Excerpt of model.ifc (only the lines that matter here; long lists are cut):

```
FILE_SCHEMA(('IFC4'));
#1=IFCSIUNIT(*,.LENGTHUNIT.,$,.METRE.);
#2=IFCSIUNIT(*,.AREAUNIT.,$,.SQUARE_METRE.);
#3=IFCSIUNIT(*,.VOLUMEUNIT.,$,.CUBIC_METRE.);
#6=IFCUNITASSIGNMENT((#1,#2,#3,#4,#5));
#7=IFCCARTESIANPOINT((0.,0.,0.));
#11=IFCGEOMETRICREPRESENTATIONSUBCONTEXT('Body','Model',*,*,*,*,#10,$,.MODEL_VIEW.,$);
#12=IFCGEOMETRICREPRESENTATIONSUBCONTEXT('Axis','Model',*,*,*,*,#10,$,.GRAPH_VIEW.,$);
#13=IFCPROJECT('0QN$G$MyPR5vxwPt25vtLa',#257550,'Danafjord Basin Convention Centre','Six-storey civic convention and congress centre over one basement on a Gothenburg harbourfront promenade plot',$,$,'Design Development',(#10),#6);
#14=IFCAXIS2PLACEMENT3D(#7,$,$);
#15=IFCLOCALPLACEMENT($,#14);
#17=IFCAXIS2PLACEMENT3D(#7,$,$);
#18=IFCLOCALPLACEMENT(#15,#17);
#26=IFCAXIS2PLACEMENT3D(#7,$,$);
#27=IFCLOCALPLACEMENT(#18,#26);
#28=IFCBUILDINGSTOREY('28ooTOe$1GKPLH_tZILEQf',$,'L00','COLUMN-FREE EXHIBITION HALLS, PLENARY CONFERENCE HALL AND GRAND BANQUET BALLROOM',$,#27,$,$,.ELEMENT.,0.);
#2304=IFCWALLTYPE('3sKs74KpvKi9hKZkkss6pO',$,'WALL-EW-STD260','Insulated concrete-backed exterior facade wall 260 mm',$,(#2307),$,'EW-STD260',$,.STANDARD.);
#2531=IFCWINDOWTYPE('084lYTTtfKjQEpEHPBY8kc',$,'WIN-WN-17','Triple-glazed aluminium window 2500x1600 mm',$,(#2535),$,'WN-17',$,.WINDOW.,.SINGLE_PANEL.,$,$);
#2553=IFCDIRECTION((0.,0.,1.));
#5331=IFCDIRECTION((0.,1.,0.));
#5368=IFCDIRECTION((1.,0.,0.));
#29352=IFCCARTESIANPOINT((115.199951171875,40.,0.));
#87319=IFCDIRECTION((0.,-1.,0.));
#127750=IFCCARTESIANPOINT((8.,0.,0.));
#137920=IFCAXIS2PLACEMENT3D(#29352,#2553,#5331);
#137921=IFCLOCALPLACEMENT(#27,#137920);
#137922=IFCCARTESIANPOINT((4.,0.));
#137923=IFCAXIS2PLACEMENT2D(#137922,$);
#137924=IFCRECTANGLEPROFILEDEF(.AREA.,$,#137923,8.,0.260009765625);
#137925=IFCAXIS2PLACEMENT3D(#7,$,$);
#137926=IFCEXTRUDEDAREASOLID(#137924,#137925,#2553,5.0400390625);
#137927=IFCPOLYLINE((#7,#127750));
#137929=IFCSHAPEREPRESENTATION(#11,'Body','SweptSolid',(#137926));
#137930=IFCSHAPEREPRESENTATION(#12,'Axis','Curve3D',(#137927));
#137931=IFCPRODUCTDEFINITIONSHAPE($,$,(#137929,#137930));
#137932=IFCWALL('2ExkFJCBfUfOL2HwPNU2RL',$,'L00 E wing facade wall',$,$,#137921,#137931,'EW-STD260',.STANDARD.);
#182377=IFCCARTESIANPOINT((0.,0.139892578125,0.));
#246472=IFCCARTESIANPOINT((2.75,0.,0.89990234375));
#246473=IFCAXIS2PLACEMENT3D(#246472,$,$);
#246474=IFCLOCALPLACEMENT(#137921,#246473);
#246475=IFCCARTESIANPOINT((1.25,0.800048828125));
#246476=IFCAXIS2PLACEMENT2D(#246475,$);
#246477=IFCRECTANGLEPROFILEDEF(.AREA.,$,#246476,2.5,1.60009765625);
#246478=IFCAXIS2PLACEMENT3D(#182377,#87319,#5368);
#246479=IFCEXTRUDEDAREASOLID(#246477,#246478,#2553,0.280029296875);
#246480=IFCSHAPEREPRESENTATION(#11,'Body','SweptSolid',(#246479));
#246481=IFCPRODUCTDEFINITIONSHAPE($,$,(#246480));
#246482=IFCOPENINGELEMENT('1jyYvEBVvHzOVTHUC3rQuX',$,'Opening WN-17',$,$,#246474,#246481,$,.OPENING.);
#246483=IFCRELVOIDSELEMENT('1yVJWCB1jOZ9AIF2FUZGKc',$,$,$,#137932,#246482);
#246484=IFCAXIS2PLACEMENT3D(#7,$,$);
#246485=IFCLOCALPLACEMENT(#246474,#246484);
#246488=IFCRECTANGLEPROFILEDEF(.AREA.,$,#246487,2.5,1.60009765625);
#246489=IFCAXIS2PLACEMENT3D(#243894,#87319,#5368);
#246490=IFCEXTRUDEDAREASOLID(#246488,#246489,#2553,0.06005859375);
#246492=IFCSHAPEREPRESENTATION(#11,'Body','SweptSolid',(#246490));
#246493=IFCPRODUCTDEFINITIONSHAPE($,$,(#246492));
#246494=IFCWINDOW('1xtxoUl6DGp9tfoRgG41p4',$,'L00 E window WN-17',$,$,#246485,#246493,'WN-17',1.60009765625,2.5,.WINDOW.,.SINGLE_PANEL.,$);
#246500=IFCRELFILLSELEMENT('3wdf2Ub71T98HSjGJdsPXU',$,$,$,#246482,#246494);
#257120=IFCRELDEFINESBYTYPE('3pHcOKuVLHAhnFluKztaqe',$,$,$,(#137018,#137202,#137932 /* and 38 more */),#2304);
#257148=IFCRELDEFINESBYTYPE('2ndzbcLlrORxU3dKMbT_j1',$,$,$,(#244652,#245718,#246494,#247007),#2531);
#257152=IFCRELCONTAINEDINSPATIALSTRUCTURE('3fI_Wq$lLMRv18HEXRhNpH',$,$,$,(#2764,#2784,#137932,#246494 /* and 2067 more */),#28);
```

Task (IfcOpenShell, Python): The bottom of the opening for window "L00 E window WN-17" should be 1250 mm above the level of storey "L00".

```python
import numpy as np
import ifcopenshell
import ifcopenshell.api.geometry
import ifcopenshell.geom
import ifcopenshell.util.element
import ifcopenshell.util.placement
import ifcopenshell.util.shape
import ifcopenshell.util.unit

model = ifcopenshell.open("model.ifc")
unit_scale = ifcopenshell.util.unit.calculate_unit_scale(model)

window = model.by_guid("1xtxoUl6DGp9tfoRgG41p4")
opening = window.FillsVoids[0].RelatingOpeningElement
storey = ifcopenshell.util.element.get_container(window, ifc_class="IfcBuildingStorey")
level = ifcopenshell.util.placement.get_local_placement(storey.ObjectPlacement)[2, 3]

# The opening's origin need not be at the sill, so measure its lowest point.
shape = ifcopenshell.geom.create_shape(ifcopenshell.geom.settings(), opening)
bottom = ifcopenshell.util.shape.get_shape_bottom_elevation(shape, shape.geometry) / unit_scale
dz = level + 1.25 - bottom

shift = np.array([0.0, 0.0, dz])
# The window is placed relative to its opening, so it follows when the opening moves.
matrix = ifcopenshell.util.placement.get_local_placement(opening.ObjectPlacement)
matrix[:3, 3] += shift
ifcopenshell.api.geometry.edit_object_placement(
    model, product=opening, matrix=matrix, is_si=False, should_transform_children=True
)

print(f"moved by {dz * unit_scale:+.3f} m")

model.write("model_updated.ifc")
```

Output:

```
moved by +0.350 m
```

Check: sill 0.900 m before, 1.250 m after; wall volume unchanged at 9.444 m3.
